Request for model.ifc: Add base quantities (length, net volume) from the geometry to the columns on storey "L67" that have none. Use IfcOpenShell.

First a look at what the model holds.

```python
import ifcopenshell
import ifcopenshell.util.element
import ifcopenshell.util.unit

model = ifcopenshell.open("model.ifc")
print(model.schema)
for unit_type in ("LENGTHUNIT", "AREAUNIT", "VOLUMEUNIT"):
    print(unit_type, ifcopenshell.util.unit.calculate_unit_scale(model, unit_type))
storey = next(s for s in model.by_type("IfcBuildingStorey") if s.Name == "L67")
columns = [e for e in ifcopenshell.util.element.get_decomposition(storey) if e.is_a("IfcColumn")]
for e in sorted(columns, key=lambda e: e.id()):
    print(e.id(), e.is_a(), e.Name, list(ifcopenshell.util.element.get_psets(e, qtos_only=True)), sep=" | ")
```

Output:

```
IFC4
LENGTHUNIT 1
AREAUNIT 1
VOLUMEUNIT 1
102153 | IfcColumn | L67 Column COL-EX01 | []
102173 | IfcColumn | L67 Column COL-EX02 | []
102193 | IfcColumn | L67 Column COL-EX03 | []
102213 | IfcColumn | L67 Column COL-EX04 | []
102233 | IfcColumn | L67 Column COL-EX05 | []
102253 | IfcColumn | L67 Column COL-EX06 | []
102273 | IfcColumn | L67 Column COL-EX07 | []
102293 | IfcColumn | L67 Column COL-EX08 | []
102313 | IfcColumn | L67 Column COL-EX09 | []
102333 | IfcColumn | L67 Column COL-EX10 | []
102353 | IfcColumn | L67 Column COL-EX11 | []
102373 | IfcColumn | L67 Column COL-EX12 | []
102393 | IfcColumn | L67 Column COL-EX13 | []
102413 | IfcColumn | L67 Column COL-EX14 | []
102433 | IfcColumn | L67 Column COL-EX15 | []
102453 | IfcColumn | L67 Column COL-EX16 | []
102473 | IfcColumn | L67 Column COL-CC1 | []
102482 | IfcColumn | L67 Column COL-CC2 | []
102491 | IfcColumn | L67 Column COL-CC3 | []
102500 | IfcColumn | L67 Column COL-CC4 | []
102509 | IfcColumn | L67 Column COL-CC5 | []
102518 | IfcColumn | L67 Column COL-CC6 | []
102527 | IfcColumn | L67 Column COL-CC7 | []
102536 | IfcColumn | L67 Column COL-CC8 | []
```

```python
import ifcopenshell
import ifcopenshell.api.pset
import ifcopenshell.geom
import ifcopenshell.util.element
import ifcopenshell.util.shape
import ifcopenshell.util.unit

model = ifcopenshell.open("model.ifc")
unit_scale = ifcopenshell.util.unit.calculate_unit_scale(model)
volume_scale = ifcopenshell.util.unit.calculate_unit_scale(model, "VOLUMEUNIT")
settings = ifcopenshell.geom.settings()

storey = next(s for s in model.by_type("IfcBuildingStorey") if s.Name == "L67")
columns = [e for e in ifcopenshell.util.element.get_decomposition(storey) if e.is_a("IfcColumn")]

for e in sorted(columns, key=lambda e: e.id()):
    if ifcopenshell.util.element.get_psets(e, qtos_only=True, should_inherit=False):
        continue
    # Geometry comes back in metres, in the element's own axes.
    shape = ifcopenshell.geom.create_shape(settings, e)
    values = {
        "Length": ifcopenshell.util.shape.get_z(shape.geometry) / unit_scale,
        "NetVolume": ifcopenshell.util.shape.get_volume(shape.geometry) / volume_scale,
    }
    qto = ifcopenshell.api.pset.add_qto(model, product=e, name="Qto_ColumnBaseQuantities")
    ifcopenshell.api.pset.edit_qto(model, qto=qto, properties=values)
    print(e.id(), {k: round(v, 3) for k, v in values.items()})

model.write("model_updated.ifc")
```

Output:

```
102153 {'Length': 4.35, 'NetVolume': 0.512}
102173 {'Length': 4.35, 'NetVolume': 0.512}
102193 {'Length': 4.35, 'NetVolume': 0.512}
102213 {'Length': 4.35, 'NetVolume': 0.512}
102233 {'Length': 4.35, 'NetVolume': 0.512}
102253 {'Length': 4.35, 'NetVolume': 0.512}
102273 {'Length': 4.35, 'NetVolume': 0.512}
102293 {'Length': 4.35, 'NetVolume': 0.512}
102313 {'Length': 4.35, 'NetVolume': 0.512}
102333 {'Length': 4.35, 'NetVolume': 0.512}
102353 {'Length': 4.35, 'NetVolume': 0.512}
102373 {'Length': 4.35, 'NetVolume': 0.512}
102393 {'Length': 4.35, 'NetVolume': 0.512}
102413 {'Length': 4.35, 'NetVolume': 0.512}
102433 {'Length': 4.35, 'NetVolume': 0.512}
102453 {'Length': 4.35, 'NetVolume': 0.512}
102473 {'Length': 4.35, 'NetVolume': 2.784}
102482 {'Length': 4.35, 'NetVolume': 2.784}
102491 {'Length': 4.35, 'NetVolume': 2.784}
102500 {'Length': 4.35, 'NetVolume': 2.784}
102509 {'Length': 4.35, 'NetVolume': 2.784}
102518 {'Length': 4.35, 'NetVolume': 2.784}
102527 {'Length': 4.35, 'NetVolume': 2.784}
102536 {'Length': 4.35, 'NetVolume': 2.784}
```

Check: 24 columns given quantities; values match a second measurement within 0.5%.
